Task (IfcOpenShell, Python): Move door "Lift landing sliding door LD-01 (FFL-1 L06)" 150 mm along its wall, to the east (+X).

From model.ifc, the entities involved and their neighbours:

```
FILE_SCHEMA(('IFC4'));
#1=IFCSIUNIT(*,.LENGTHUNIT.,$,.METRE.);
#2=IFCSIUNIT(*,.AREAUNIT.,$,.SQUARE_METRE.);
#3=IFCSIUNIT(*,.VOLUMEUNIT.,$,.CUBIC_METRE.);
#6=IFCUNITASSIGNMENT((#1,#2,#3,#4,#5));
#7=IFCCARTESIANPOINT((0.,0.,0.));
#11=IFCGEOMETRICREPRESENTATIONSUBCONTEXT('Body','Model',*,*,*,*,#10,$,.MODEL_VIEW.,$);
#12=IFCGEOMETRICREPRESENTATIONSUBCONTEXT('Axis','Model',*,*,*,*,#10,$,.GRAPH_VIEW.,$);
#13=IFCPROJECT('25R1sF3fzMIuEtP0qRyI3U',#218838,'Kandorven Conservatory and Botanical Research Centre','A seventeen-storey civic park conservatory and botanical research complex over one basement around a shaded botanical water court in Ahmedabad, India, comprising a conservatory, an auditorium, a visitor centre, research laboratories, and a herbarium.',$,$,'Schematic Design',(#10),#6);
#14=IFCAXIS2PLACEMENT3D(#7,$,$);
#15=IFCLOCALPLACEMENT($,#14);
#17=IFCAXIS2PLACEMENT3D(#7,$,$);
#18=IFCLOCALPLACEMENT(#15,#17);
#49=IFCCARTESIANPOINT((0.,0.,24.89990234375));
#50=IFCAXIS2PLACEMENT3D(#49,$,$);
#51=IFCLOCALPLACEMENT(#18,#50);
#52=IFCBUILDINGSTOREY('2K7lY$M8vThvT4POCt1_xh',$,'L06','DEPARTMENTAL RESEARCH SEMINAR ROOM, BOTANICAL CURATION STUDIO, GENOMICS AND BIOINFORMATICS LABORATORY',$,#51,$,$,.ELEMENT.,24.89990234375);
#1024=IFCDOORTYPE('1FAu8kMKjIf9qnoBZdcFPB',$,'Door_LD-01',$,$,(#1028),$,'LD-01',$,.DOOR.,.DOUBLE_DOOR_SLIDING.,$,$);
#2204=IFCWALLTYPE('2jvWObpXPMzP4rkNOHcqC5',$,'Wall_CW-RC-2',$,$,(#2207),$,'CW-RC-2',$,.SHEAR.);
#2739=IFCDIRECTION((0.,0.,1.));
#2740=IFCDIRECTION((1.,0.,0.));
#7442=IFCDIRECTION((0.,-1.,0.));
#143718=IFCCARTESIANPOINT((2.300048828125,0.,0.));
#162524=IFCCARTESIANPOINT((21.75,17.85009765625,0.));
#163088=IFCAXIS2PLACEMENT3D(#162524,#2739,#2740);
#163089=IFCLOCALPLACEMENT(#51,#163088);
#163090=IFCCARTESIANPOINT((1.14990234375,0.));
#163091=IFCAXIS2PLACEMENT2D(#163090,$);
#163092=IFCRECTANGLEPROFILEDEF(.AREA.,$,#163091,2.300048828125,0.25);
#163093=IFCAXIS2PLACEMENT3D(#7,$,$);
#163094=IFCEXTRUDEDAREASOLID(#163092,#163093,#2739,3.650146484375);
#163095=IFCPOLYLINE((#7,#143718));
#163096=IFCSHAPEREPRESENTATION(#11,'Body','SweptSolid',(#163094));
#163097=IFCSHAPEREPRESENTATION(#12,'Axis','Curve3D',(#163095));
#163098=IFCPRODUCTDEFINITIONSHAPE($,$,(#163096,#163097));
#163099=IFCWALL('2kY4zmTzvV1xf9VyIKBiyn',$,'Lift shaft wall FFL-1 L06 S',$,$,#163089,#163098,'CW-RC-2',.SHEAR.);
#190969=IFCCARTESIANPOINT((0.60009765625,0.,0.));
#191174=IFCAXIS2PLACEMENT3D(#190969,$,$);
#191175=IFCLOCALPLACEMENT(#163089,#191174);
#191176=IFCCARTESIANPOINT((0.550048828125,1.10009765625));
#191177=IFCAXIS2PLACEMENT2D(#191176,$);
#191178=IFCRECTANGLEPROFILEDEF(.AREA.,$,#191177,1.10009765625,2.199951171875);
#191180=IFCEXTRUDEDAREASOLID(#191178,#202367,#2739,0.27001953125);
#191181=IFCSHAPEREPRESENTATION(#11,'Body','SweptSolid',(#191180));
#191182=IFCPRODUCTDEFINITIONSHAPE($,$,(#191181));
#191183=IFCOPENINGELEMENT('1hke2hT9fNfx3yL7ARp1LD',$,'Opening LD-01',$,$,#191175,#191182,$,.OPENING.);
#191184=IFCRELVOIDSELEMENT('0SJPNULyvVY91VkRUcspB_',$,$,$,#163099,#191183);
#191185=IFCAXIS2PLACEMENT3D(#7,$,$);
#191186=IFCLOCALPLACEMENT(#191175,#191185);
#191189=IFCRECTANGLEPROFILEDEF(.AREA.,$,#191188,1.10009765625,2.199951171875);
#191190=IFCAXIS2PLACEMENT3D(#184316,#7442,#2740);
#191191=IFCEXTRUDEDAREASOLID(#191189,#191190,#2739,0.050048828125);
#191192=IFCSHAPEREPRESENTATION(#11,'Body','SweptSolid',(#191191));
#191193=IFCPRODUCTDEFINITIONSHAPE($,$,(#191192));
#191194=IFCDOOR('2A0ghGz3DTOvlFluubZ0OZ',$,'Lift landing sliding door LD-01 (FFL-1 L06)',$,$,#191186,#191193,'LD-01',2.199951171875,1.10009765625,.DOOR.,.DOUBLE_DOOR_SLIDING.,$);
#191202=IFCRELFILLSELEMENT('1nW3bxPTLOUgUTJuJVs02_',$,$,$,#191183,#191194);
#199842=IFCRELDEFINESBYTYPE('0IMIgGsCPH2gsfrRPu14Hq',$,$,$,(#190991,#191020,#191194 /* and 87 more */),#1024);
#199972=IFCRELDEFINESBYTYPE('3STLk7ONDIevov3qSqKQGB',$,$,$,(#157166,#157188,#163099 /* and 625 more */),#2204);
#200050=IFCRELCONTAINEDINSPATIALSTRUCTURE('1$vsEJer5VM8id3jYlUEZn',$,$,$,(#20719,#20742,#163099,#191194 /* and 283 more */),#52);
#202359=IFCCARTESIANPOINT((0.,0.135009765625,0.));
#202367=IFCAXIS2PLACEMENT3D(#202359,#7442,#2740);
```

```python
import ifcopenshell
import ifcopenshell.api.geometry
import ifcopenshell.util.placement

model = ifcopenshell.open("model.ifc")

door = model.by_guid("2A0ghGz3DTOvlFluubZ0OZ")
opening = door.FillsVoids[0].RelatingOpeningElement
wall = opening.VoidsElements[0].RelatingBuildingElement

wall_matrix = ifcopenshell.util.placement.get_local_placement(wall.ObjectPlacement)
shift = wall_matrix[:3, 0] * 0.15
before = ifcopenshell.util.placement.get_local_placement(door.ObjectPlacement)[:3, 3].copy()

# The door is placed relative to its opening, so it follows when the opening moves.
matrix = ifcopenshell.util.placement.get_local_placement(opening.ObjectPlacement)
matrix[:3, 3] += shift
ifcopenshell.api.geometry.edit_object_placement(
    model, product=opening, matrix=matrix, is_si=False, should_transform_children=True
)

after = ifcopenshell.util.placement.get_local_placement(door.ObjectPlacement)[:3, 3]
print("door moved by", (after - before).round(3) + 0.0)

model.write("model_edited.ifc")
```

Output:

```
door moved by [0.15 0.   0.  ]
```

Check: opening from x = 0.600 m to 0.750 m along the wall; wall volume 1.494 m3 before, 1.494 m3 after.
